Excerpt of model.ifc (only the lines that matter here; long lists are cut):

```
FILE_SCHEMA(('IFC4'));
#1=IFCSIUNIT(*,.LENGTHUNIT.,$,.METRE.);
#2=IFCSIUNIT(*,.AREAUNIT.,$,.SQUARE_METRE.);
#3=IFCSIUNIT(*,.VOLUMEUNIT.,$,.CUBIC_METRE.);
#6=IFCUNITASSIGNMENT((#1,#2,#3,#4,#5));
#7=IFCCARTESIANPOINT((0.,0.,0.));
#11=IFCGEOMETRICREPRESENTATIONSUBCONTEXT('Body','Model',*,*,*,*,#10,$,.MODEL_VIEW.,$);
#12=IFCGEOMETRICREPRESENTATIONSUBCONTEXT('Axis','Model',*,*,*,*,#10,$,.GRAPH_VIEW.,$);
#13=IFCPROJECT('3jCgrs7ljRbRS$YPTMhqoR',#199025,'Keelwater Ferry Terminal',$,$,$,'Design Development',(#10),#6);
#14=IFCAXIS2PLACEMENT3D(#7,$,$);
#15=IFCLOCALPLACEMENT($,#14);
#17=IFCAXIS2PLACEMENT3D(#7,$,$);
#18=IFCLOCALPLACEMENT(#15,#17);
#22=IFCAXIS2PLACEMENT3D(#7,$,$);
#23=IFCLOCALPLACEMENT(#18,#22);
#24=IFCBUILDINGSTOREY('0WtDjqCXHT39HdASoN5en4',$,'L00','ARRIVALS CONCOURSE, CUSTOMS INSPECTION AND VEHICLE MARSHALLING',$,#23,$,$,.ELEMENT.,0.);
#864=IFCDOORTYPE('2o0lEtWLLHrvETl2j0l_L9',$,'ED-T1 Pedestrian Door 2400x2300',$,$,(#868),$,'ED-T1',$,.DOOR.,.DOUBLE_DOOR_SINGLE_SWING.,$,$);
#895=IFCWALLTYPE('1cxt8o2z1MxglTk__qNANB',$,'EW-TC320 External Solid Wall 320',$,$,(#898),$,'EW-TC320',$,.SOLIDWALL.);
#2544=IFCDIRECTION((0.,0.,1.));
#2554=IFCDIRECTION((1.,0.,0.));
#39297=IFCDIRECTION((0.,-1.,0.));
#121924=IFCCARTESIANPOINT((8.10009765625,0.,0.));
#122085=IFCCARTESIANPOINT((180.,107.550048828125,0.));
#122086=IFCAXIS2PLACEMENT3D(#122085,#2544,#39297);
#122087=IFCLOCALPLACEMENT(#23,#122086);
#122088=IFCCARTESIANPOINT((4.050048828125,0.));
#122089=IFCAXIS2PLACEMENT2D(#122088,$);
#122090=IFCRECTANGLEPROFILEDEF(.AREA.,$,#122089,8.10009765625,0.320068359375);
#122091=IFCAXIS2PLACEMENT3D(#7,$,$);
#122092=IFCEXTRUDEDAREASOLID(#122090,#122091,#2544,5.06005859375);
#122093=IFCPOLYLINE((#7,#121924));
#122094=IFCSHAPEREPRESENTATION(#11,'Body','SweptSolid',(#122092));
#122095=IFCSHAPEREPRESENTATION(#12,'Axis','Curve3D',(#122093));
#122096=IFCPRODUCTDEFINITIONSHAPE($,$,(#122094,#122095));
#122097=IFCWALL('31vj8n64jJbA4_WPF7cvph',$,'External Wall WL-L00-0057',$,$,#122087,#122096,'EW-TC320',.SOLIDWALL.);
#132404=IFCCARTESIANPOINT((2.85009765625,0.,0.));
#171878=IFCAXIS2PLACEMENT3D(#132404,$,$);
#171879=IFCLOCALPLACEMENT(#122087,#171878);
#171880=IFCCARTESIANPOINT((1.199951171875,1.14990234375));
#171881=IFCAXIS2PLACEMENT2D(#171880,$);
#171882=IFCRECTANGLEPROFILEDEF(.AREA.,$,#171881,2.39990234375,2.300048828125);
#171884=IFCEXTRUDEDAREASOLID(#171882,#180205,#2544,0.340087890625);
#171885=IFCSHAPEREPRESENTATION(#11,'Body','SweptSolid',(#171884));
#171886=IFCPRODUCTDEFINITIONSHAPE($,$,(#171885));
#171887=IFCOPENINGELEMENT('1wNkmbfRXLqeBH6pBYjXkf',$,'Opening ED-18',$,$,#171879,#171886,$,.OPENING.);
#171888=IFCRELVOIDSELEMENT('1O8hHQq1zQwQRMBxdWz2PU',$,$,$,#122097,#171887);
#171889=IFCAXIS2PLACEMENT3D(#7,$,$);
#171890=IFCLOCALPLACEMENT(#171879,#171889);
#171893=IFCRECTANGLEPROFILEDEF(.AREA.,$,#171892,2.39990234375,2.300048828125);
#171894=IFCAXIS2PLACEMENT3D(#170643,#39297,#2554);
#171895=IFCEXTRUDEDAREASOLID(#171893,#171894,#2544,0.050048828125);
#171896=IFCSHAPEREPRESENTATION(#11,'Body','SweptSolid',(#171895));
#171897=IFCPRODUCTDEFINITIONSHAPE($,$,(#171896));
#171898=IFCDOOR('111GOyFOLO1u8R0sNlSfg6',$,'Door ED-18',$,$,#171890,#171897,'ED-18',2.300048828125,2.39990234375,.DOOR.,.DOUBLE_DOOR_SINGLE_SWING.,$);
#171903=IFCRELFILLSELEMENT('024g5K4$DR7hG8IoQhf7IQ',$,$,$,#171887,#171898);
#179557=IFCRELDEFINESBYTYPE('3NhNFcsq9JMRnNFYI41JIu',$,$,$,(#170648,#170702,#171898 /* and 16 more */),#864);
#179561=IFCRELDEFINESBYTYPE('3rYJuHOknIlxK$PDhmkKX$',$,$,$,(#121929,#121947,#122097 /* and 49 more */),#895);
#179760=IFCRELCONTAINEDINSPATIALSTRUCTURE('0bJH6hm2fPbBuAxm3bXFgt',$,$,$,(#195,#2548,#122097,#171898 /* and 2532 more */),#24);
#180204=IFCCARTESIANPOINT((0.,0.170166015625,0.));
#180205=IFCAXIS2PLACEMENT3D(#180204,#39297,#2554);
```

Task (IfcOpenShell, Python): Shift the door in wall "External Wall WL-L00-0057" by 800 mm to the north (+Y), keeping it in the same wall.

```python
import ifcopenshell
import ifcopenshell.api.geometry
import ifcopenshell.util.placement

model = ifcopenshell.open("model.ifc")

door = model.by_id(171898)
opening = door.FillsVoids[0].RelatingOpeningElement
wall = opening.VoidsElements[0].RelatingBuildingElement

wall_matrix = ifcopenshell.util.placement.get_local_placement(wall.ObjectPlacement)
shift = wall_matrix[:3, 0] * -0.8
before = ifcopenshell.util.placement.get_local_placement(door.ObjectPlacement)[:3, 3].copy()

# The door is placed relative to its opening, so it follows when the opening moves.
matrix = ifcopenshell.util.placement.get_local_placement(opening.ObjectPlacement)
matrix[:3, 3] += shift
ifcopenshell.api.geometry.edit_object_placement(
    model, product=opening, matrix=matrix, is_si=False, should_transform_children=True
)

after = ifcopenshell.util.placement.get_local_placement(door.ObjectPlacement)[:3, 3]
print("door moved by", (after - before).round(3) + 0.0)

model.write("model_edited.ifc")
```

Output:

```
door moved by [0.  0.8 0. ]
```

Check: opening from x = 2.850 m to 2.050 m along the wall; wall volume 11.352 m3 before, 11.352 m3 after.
